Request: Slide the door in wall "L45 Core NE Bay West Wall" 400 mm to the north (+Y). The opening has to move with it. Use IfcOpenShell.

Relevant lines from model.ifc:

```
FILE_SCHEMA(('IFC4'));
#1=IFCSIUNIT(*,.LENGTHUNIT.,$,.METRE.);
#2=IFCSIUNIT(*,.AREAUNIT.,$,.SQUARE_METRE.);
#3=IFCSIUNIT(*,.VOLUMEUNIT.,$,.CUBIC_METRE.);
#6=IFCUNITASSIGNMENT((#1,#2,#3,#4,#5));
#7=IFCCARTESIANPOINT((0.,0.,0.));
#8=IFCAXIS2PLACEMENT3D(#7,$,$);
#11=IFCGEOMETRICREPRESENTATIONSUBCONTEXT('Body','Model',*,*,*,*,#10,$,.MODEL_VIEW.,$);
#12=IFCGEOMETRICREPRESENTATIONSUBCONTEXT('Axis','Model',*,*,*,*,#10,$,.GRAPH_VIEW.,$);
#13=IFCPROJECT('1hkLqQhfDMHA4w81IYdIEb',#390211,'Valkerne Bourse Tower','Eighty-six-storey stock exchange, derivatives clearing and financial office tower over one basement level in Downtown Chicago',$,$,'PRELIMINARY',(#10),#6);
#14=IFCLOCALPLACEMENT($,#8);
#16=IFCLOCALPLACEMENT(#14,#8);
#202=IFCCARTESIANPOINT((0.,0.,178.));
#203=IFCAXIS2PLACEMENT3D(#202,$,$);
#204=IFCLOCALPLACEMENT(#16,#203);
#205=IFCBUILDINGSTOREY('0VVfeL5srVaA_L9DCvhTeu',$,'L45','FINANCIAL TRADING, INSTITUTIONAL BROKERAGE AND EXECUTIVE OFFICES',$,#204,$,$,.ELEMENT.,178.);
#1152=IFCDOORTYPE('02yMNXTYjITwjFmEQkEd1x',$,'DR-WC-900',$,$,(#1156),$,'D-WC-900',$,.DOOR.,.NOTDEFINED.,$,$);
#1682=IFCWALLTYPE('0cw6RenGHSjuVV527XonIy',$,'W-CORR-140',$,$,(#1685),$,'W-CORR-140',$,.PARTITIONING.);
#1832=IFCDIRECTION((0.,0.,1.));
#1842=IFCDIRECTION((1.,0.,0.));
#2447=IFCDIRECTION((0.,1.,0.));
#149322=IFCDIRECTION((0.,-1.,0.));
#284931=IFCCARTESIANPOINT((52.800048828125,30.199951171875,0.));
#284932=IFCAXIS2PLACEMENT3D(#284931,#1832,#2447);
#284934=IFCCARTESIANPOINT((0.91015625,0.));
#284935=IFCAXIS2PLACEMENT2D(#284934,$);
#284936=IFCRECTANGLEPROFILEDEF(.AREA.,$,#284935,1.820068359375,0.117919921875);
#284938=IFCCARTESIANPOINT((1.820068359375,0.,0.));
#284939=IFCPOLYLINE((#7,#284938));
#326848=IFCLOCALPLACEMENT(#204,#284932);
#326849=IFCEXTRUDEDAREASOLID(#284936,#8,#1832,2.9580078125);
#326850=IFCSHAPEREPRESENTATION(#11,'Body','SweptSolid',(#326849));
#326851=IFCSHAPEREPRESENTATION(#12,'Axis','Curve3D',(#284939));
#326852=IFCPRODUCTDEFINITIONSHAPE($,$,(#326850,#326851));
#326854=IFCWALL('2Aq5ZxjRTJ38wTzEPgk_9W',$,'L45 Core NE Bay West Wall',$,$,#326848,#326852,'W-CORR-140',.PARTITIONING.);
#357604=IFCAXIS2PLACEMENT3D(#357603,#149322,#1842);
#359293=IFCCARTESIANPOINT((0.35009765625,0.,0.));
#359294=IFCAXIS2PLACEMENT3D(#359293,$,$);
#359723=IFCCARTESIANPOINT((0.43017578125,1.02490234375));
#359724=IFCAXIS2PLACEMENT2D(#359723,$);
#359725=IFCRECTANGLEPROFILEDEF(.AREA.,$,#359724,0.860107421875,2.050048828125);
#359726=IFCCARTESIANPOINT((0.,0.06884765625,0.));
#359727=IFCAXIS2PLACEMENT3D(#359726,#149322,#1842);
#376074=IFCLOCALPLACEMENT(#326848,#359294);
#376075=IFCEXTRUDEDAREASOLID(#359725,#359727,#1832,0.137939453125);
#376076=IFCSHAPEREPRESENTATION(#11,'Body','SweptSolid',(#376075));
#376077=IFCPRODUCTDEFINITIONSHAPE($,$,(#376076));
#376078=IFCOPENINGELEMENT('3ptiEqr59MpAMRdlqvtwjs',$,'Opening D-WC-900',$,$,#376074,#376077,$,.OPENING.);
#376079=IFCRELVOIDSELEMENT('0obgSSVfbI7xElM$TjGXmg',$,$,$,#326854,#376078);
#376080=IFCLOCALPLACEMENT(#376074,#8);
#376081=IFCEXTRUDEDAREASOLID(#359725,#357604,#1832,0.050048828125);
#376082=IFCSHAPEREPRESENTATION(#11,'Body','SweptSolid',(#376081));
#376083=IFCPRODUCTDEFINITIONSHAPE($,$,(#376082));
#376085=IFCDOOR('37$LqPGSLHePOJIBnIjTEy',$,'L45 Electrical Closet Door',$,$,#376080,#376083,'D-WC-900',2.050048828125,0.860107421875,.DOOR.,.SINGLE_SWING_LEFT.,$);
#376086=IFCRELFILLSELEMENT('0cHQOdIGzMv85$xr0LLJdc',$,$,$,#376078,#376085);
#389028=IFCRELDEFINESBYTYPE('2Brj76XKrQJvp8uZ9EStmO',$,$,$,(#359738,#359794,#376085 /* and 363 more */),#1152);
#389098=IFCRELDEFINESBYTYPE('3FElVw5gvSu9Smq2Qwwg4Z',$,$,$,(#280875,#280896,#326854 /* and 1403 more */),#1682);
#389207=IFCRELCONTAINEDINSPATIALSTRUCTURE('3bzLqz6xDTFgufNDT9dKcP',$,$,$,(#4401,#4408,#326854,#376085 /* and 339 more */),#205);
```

```python
import ifcopenshell
import ifcopenshell.api.geometry
import ifcopenshell.util.placement
import ifcopenshell.util.unit

model = ifcopenshell.open("model.ifc")
unit_scale = ifcopenshell.util.unit.calculate_unit_scale(model)

door = model.by_guid("37$LqPGSLHePOJIBnIjTEy")
opening = door.FillsVoids[0].RelatingOpeningElement
wall = opening.VoidsElements[0].RelatingBuildingElement

wall_matrix = ifcopenshell.util.placement.get_local_placement(wall.ObjectPlacement)
shift = wall_matrix[:3, 0] * 0.4 / unit_scale
before = ifcopenshell.util.placement.get_local_placement(door.ObjectPlacement)[:3, 3].copy()

# The door is placed relative to its opening, so it follows when the opening moves.
matrix = ifcopenshell.util.placement.get_local_placement(opening.ObjectPlacement)
matrix[:3, 3] += shift
ifcopenshell.api.geometry.edit_object_placement(
    model, product=opening, matrix=matrix, is_si=False, should_transform_children=True
)

after = ifcopenshell.util.placement.get_local_placement(door.ObjectPlacement)[:3, 3]
print("door moved by", (after - before).round(3) + 0.0)

model.write("model_edited.ifc")
```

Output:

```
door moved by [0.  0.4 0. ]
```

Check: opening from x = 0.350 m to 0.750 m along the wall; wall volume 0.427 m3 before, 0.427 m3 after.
